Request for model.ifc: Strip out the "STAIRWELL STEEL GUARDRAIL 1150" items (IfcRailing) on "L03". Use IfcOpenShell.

First a look at what the model holds.

```python
import ifcopenshell
import ifcopenshell.util.element

model = ifcopenshell.open("model.ifc")
print(model.schema)
storey = next(s for s in model.by_type("IfcBuildingStorey") if s.Name == "L03")
railings = [e for e in ifcopenshell.util.element.get_decomposition(storey) if e.is_a("IfcRailing")]
seen = {}
for e in railings:
    element_type = ifcopenshell.util.element.get_type(e)
    name = element_type.Name if element_type not in (None, e) else None
    seen[name] = seen.get(name, 0) + 1
for name, count in sorted(seen.items(), key=str):
    print(count, "x", name)
```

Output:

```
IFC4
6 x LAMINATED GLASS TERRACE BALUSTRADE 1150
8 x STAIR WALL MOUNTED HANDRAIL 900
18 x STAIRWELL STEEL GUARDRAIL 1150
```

```python
import ifcopenshell
import ifcopenshell.api.root
import ifcopenshell.util.element

model = ifcopenshell.open("model.ifc")

storey = next(s for s in model.by_type("IfcBuildingStorey") if s.Name == "L03")
railings = [e for e in ifcopenshell.util.element.get_decomposition(storey) if e.is_a("IfcRailing")]
targets = [e for e in railings if (t := ifcopenshell.util.element.get_type(e)) not in (None, e) and t.Name == "STAIRWELL STEEL GUARDRAIL 1150"]

for e in targets:
    ifcopenshell.api.root.remove_product(model, product=e)
print(len(targets), "removed")

model.write("model_edited.ifc")
```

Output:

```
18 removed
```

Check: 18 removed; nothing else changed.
